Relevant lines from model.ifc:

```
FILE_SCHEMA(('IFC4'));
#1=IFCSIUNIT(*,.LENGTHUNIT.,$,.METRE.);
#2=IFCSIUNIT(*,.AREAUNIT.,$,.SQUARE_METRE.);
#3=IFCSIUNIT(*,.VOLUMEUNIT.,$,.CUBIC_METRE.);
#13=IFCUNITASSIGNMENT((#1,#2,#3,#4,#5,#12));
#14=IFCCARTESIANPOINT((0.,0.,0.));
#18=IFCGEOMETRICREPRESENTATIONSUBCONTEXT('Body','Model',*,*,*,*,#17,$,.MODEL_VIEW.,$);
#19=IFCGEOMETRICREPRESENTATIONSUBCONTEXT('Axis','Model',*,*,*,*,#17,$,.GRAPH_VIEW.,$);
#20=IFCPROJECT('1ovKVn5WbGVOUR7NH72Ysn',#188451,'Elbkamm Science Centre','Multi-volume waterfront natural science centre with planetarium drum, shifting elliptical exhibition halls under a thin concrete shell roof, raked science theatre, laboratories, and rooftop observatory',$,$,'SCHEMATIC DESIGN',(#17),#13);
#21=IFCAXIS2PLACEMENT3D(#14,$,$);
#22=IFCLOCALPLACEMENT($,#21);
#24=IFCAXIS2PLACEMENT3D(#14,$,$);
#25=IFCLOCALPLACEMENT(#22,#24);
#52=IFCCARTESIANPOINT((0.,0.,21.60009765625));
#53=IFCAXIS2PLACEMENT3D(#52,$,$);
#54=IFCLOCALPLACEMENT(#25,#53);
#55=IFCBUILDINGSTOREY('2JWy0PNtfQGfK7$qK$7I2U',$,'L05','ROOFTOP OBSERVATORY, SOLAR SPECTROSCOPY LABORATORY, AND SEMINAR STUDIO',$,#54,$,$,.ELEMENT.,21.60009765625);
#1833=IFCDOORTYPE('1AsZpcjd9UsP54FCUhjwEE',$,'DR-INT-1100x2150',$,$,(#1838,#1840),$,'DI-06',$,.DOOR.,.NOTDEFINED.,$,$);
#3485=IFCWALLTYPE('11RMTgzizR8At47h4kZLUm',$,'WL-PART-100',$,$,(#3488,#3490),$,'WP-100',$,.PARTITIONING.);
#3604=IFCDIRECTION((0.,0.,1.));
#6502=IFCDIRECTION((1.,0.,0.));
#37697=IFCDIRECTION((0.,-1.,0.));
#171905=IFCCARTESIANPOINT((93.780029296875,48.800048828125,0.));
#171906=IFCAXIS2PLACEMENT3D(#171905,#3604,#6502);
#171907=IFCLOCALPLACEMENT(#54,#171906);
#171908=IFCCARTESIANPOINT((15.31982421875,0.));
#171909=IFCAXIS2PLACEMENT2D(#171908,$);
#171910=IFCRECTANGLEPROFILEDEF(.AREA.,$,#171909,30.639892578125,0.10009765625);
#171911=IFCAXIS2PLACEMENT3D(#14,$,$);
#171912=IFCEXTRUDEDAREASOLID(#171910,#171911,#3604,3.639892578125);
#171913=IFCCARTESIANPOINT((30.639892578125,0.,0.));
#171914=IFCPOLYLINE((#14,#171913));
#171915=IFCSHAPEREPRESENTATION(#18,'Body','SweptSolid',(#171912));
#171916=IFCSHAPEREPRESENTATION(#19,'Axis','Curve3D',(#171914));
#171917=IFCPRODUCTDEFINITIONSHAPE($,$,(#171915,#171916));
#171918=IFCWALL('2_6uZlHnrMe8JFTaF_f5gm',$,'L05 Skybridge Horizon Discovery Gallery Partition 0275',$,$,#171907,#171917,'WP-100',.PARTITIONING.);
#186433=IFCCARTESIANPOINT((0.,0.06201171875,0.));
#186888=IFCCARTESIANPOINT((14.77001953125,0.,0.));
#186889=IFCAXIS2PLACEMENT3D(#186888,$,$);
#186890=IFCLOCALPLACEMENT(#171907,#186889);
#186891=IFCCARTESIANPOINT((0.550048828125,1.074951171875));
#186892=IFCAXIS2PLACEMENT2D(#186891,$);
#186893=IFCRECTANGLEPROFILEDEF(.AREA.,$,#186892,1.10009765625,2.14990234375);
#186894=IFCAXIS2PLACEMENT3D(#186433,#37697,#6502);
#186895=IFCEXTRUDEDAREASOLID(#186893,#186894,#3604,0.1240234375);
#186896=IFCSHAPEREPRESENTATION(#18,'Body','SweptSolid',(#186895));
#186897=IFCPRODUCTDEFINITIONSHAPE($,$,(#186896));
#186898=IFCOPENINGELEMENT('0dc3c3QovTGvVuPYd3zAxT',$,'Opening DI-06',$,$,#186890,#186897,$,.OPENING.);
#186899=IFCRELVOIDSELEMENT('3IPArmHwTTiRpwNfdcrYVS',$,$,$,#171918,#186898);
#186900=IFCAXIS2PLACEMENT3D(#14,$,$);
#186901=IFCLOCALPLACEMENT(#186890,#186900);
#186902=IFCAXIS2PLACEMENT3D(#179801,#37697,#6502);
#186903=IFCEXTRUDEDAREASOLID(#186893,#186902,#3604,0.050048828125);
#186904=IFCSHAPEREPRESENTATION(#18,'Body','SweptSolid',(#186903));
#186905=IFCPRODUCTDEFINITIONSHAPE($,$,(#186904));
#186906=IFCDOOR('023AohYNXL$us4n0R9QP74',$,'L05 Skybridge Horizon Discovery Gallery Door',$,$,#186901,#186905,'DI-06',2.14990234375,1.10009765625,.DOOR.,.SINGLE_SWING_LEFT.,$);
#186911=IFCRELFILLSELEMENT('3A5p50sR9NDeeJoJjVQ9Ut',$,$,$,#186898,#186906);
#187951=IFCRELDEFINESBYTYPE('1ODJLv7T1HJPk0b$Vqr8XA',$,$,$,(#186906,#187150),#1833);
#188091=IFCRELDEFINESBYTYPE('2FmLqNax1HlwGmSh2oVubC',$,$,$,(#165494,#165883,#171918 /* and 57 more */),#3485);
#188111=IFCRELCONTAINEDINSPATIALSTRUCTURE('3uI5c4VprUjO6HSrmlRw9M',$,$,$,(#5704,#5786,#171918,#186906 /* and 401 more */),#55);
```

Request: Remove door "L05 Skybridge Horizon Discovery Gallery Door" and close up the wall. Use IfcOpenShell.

```python
import ifcopenshell
import ifcopenshell.api.feature
import ifcopenshell.api.root
import ifcopenshell.geom
import ifcopenshell.util.shape

model = ifcopenshell.open("model.ifc")
settings = ifcopenshell.geom.settings()


def volume(element):
    """Net volume in cubic metres, openings subtracted."""
    shape = ifcopenshell.geom.create_shape(settings, element)
    return ifcopenshell.util.shape.get_volume(shape.geometry)


door = model.by_guid("023AohYNXL$us4n0R9QP74")
opening = door.FillsVoids[0].RelatingOpeningElement
wall = opening.VoidsElements[0].RelatingBuildingElement
before = volume(wall)

ifcopenshell.api.root.remove_product(model, product=door)
ifcopenshell.api.feature.remove_feature(model, feature=opening)

after = volume(wall)

print(f"wall volume {before:.3f} -> {after:.3f} m3")

model.write("model_edited.ifc")
```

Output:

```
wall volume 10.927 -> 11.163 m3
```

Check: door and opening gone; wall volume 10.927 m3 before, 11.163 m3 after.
